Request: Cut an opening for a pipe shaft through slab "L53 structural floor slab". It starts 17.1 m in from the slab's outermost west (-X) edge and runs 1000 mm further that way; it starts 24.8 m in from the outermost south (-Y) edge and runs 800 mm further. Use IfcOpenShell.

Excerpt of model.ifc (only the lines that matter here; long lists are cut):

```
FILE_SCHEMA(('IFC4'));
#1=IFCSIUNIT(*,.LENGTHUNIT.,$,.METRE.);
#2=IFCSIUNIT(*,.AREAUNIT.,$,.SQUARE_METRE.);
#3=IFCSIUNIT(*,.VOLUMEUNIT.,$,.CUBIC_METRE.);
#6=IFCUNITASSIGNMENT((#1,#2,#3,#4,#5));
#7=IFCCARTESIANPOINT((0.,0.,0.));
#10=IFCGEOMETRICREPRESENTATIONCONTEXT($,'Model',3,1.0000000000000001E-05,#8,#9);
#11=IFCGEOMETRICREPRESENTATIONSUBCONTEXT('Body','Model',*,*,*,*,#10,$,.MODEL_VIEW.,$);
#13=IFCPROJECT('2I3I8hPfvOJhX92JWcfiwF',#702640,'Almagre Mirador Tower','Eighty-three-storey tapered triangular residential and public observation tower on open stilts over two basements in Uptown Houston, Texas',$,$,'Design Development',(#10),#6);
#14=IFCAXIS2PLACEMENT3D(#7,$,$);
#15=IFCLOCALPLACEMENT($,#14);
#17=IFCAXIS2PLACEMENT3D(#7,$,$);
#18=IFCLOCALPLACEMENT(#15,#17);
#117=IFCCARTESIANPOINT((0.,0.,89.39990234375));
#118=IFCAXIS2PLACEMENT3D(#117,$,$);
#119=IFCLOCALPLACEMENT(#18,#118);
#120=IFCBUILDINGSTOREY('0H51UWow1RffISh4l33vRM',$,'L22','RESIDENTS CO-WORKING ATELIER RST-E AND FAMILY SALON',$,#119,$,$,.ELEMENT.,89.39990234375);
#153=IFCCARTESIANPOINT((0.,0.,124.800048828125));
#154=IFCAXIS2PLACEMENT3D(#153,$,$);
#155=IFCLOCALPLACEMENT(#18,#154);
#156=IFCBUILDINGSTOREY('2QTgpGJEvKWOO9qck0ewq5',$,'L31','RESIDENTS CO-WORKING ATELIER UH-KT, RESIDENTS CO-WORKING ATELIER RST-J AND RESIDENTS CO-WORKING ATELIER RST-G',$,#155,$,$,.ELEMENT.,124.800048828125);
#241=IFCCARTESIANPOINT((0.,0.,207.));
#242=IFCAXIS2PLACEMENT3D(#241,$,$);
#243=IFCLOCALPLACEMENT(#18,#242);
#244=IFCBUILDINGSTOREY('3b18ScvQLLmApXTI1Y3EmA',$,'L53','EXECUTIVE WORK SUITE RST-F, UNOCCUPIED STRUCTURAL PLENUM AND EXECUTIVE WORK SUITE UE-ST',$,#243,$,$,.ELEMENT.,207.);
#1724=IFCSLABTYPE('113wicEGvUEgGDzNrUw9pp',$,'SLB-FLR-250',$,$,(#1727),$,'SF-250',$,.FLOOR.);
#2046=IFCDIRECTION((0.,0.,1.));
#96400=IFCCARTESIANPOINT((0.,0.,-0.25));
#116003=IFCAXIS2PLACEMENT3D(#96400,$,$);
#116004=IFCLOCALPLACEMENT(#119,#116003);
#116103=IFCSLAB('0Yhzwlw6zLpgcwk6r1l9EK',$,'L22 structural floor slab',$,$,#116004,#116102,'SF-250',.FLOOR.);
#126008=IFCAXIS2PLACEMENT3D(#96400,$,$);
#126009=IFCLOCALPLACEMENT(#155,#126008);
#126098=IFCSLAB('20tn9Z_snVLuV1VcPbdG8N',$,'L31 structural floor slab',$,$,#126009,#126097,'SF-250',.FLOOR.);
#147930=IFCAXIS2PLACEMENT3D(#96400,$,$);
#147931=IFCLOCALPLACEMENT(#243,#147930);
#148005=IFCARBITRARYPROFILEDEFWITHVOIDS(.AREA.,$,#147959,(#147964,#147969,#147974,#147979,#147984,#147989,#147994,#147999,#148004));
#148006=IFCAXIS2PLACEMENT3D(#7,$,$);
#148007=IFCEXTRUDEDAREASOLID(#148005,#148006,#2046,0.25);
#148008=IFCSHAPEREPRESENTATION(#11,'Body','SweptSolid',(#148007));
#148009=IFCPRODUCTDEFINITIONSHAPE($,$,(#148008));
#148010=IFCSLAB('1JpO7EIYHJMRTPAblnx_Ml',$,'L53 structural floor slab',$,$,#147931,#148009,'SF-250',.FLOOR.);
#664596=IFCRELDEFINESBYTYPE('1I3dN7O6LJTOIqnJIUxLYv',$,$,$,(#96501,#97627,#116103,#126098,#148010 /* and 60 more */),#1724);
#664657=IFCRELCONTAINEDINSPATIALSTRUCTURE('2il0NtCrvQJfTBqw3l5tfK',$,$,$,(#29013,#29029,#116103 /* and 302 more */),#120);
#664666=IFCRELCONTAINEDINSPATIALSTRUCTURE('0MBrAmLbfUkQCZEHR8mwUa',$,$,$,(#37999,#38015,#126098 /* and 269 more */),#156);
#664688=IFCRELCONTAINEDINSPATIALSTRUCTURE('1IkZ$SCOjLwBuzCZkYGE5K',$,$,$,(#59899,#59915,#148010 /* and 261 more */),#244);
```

```python
import numpy as np
import ifcopenshell
import ifcopenshell.api.feature
import ifcopenshell.api.geometry
import ifcopenshell.api.root
import ifcopenshell.geom
import ifcopenshell.util.placement
import ifcopenshell.util.representation
import ifcopenshell.util.shape
import ifcopenshell.util.unit

model = ifcopenshell.open("model.ifc")
unit_scale = ifcopenshell.util.unit.calculate_unit_scale(model)
settings = ifcopenshell.geom.settings()


def volume(element):
    """Net volume in cubic metres, openings subtracted."""
    shape = ifcopenshell.geom.create_shape(settings, element)
    return ifcopenshell.util.shape.get_volume(shape.geometry)


slab = model.by_id(148010)
before = volume(slab)

# Extent in the slab's own axes, in metres. The edges named are its -X and -Y sides.
slab_shape = ifcopenshell.geom.create_shape(settings, slab)
vertices = ifcopenshell.util.shape.get_vertices(slab_shape.geometry)
x_min, y_min, bottom = vertices.min(axis=0)
top = vertices[:, 2].max()

opening = ifcopenshell.api.root.create_entity(model, ifc_class="IfcOpeningElement", name="Pipe shaft opening", predefined_type="OPENING")
context = ifcopenshell.util.representation.get_context(model, "Model", "Body", "MODEL_VIEW")
width, depth = 1, 0.8
outline = [(0.0, 0.0), (width, 0.0), (width, depth), (0.0, depth), (0.0, 0.0)]
# Overshoot both faces by 50 mm so the cut is clean.
shape = ifcopenshell.api.geometry.add_slab_representation(
    model, context=context, depth=top - bottom + 0.1, polyline=outline
)
ifcopenshell.api.geometry.assign_representation(model, product=opening, representation=shape)

matrix = ifcopenshell.util.placement.get_local_placement(slab.ObjectPlacement)
matrix[:, 3] = matrix @ np.append(np.array([x_min + 17.1, y_min + 24.8, bottom - 0.05]) / unit_scale, 1.0)
ifcopenshell.api.geometry.edit_object_placement(model, product=opening, matrix=matrix, is_si=False)
ifcopenshell.api.feature.add_feature(model, feature=opening, element=slab)

after = volume(slab)

print(f"slab volume {before:.3f} -> {after:.3f} m3")

model.write("model_updated.ifc")
```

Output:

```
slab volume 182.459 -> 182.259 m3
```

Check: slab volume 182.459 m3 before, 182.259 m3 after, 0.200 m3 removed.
